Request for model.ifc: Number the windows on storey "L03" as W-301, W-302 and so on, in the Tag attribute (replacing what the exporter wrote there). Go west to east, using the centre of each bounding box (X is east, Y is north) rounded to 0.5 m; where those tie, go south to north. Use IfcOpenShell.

First a look at what the model holds.

```python
import ifcopenshell
import ifcopenshell.util.element
import ifcopenshell.util.placement

model = ifcopenshell.open("model.ifc")
print(model.schema)
storey = next(s for s in model.by_type("IfcBuildingStorey") if s.Name == "L03")
windows = [e for e in ifcopenshell.util.element.get_decomposition(storey) if e.is_a("IfcWindow")]
for e in sorted(windows, key=lambda e: e.id()):
    origin = ifcopenshell.util.placement.get_local_placement(e.ObjectPlacement)[:3, 3]
    print(e.id(), e.Tag, e.Name, origin.round(2) + 0.0, sep=" | ")
```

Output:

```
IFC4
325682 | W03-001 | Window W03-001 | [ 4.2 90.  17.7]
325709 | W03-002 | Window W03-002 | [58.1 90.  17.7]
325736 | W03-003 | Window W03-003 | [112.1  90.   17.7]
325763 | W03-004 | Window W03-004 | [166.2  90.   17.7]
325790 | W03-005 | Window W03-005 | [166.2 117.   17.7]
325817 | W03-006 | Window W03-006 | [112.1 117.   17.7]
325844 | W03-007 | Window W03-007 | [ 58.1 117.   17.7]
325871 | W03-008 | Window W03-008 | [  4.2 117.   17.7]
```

```python
import ifcopenshell
import ifcopenshell.geom
import ifcopenshell.util.element
import ifcopenshell.util.shape

model = ifcopenshell.open("model.ifc")
settings = ifcopenshell.geom.settings()
settings.set("use-world-coords", True)


def centre(element):
    shape = ifcopenshell.geom.create_shape(settings, element)
    return ifcopenshell.util.shape.get_bbox_centroid(shape.geometry)


storey = next(s for s in model.by_type("IfcBuildingStorey") if s.Name == "L03")
windows = [e for e in ifcopenshell.util.element.get_decomposition(storey) if e.is_a("IfcWindow")]

# Insertion points can sit at a corner or the storey origin, so sort by the geometry (in metres).
centres = {e: centre(e) for e in windows}
windows.sort(key=lambda e: (round(centres[e][0] / 0.5), centres[e][1]))

for i, e in enumerate(windows, start=1):
    number = f"W-3{i:02d}"
    e.Tag = number
    print(e.id(), number)

model.write("model_updated.ifc")
```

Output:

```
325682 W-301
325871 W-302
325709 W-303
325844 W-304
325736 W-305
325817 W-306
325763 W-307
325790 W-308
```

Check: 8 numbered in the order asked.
